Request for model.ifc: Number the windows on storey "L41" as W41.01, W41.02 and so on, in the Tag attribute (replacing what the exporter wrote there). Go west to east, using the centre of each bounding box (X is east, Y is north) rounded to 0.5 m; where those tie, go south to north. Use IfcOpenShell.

First a look at what the model holds.

```python
import ifcopenshell
import ifcopenshell.util.element
import ifcopenshell.util.placement

model = ifcopenshell.open("model.ifc")
print(model.schema)
storey = next(s for s in model.by_type("IfcBuildingStorey") if s.Name == "L41")
windows = [e for e in ifcopenshell.util.element.get_decomposition(storey) if e.is_a("IfcWindow")]
for e in sorted(windows, key=lambda e: e.id()):
    origin = ifcopenshell.util.placement.get_local_placement(e.ObjectPlacement)[:3, 3]
    print(e.id(), e.Tag, e.Name, origin.round(2) + 0.0, sep=" | ")
```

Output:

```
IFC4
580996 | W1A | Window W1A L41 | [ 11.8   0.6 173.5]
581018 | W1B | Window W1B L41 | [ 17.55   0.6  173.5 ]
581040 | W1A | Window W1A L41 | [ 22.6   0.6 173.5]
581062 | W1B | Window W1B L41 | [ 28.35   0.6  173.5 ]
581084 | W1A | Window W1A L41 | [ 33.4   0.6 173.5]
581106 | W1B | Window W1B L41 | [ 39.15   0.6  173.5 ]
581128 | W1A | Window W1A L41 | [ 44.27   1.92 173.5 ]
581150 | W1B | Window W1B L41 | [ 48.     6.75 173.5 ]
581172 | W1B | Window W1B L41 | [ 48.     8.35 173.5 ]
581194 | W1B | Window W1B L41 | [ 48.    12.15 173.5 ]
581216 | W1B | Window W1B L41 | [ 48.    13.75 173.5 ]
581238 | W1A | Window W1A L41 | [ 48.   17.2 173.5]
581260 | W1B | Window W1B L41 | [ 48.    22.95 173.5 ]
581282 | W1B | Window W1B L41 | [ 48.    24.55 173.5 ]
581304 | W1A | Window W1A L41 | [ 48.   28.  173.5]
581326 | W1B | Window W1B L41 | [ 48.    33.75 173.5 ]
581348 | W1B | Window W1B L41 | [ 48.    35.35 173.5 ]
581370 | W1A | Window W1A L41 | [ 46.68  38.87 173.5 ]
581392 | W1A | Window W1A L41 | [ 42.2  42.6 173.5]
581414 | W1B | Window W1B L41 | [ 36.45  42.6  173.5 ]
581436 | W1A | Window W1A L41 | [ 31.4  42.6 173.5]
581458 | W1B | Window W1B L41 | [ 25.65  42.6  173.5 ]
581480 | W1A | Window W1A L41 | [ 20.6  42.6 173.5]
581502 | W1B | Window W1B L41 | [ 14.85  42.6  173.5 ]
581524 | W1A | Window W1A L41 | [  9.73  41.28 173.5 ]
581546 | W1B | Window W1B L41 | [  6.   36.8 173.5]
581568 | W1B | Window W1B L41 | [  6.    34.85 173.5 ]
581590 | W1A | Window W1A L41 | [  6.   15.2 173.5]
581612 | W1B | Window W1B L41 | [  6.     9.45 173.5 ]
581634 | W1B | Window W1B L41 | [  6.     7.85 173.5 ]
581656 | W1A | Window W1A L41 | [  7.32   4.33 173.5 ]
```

```python
import ifcopenshell
import ifcopenshell.geom
import ifcopenshell.util.element
import ifcopenshell.util.shape

model = ifcopenshell.open("model.ifc")
settings = ifcopenshell.geom.settings()
settings.set("use-world-coords", True)


def centre(element):
    shape = ifcopenshell.geom.create_shape(settings, element)
    return ifcopenshell.util.shape.get_bbox_centroid(shape.geometry)


storey = next(s for s in model.by_type("IfcBuildingStorey") if s.Name == "L41")
windows = [e for e in ifcopenshell.util.element.get_decomposition(storey) if e.is_a("IfcWindow")]

# Insertion points can sit at a corner or the storey origin, so sort by the geometry (in metres).
centres = {e: centre(e) for e in windows}
windows.sort(key=lambda e: (round(centres[e][0] / 0.5), centres[e][1]))

for i, e in enumerate(windows, start=1):
    number = f"W41.{i:02d}"
    e.Tag = number
    print(e.id(), number)

model.write("model_updated.ifc")
```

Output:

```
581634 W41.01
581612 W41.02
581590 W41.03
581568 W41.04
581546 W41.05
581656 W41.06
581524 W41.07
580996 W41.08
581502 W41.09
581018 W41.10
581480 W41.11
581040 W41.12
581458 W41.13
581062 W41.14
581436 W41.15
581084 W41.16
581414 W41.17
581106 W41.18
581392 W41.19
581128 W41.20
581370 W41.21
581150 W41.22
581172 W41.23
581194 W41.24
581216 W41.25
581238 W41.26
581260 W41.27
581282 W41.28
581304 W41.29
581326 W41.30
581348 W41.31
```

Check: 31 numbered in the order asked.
